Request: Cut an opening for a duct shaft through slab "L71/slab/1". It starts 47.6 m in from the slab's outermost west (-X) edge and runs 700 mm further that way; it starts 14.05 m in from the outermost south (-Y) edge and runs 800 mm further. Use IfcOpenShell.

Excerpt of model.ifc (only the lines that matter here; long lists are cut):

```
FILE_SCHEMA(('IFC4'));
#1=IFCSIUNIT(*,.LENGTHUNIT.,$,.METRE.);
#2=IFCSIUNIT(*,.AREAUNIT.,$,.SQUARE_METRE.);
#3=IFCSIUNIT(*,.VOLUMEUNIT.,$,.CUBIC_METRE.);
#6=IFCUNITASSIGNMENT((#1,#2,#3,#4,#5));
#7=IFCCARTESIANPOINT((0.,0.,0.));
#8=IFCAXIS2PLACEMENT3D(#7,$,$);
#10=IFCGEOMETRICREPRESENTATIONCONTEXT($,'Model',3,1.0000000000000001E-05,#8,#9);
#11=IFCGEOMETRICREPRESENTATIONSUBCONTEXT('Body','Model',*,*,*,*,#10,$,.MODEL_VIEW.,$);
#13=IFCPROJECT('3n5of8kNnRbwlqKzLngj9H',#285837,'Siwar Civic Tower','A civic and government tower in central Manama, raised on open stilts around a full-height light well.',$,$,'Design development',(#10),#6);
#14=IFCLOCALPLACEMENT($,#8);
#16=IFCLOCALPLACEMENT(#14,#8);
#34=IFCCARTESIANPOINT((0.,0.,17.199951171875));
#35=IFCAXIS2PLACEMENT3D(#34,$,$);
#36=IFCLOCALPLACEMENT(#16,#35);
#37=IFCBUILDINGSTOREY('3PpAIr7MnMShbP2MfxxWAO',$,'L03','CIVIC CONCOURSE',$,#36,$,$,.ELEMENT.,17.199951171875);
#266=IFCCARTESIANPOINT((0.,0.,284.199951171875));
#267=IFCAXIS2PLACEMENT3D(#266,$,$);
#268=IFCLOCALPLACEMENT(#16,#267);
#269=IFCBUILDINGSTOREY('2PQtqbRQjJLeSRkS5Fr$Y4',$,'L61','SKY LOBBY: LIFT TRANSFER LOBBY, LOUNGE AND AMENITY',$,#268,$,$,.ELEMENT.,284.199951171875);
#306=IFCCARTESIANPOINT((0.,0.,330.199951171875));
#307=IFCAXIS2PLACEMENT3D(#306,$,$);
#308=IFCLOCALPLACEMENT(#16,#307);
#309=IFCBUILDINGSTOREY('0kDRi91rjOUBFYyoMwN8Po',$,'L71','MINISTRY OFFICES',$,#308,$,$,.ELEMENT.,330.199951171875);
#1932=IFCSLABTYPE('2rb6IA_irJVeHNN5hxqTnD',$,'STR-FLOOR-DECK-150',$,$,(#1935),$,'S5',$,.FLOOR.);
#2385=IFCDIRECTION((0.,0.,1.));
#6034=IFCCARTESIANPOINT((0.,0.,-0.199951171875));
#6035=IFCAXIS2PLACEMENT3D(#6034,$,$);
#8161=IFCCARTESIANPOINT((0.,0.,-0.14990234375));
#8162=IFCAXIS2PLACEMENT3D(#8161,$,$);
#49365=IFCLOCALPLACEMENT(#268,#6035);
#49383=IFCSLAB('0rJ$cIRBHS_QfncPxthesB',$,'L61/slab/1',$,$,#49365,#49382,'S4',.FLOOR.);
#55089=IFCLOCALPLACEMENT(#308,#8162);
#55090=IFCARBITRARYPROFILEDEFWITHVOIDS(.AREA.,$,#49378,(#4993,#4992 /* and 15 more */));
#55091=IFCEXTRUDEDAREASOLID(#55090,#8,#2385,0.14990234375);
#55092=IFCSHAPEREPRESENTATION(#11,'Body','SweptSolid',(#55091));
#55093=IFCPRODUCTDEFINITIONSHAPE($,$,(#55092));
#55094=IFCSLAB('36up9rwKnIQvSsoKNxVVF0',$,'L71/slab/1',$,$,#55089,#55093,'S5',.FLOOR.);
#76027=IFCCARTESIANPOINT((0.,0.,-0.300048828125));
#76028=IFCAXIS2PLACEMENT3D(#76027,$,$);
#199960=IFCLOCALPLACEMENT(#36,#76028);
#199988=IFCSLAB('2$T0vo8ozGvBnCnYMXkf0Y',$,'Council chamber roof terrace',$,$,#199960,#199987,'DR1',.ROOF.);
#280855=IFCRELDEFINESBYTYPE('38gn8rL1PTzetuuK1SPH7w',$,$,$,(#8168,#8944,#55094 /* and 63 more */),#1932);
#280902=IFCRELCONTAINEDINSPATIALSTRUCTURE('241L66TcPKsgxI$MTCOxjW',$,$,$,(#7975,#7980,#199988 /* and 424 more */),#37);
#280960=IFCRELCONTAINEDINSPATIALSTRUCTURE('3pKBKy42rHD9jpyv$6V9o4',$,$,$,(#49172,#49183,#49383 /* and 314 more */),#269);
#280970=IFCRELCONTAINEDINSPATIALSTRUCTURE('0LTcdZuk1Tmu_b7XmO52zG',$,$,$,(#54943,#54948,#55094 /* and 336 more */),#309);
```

```python
import numpy as np
import ifcopenshell
import ifcopenshell.api.feature
import ifcopenshell.api.geometry
import ifcopenshell.api.root
import ifcopenshell.geom
import ifcopenshell.util.placement
import ifcopenshell.util.representation
import ifcopenshell.util.shape
import ifcopenshell.util.unit

model = ifcopenshell.open("model.ifc")
unit_scale = ifcopenshell.util.unit.calculate_unit_scale(model)
settings = ifcopenshell.geom.settings()


def volume(element):
    """Net volume in cubic metres, openings subtracted."""
    shape = ifcopenshell.geom.create_shape(settings, element)
    return ifcopenshell.util.shape.get_volume(shape.geometry)


slab = model.by_id(55094)
before = volume(slab)

# Extent in the slab's own axes, in metres. The edges named are its -X and -Y sides.
slab_shape = ifcopenshell.geom.create_shape(settings, slab)
vertices = ifcopenshell.util.shape.get_vertices(slab_shape.geometry)
x_min, y_min, bottom = vertices.min(axis=0)
top = vertices[:, 2].max()

opening = ifcopenshell.api.root.create_entity(model, ifc_class="IfcOpeningElement", name="Duct shaft opening", predefined_type="OPENING")
context = ifcopenshell.util.representation.get_context(model, "Model", "Body", "MODEL_VIEW")
width, depth = 0.7, 0.8
outline = [(0.0, 0.0), (width, 0.0), (width, depth), (0.0, depth), (0.0, 0.0)]
# Overshoot both faces by 50 mm so the cut is clean.
shape = ifcopenshell.api.geometry.add_slab_representation(
    model, context=context, depth=top - bottom + 0.1, polyline=outline
)
ifcopenshell.api.geometry.assign_representation(model, product=opening, representation=shape)

matrix = ifcopenshell.util.placement.get_local_placement(slab.ObjectPlacement)
matrix[:, 3] = matrix @ np.append(np.array([x_min + 47.6, y_min + 14.05, bottom - 0.05]) / unit_scale, 1.0)
ifcopenshell.api.geometry.edit_object_placement(model, product=opening, matrix=matrix, is_si=False)
ifcopenshell.api.feature.add_feature(model, feature=opening, element=slab)

after = volume(slab)

print(f"slab volume {before:.3f} -> {after:.3f} m3")

model.write("model-out.ifc")
```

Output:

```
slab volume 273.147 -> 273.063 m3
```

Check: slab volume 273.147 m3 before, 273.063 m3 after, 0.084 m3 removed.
